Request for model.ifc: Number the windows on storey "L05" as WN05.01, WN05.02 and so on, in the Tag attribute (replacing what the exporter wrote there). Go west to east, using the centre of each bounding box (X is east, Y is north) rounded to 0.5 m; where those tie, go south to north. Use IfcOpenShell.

First a look at what the model holds.

```python
import ifcopenshell
import ifcopenshell.util.element
import ifcopenshell.util.placement

model = ifcopenshell.open("model.ifc")
print(model.schema)
storey = next(s for s in model.by_type("IfcBuildingStorey") if s.Name == "L05")
windows = [e for e in ifcopenshell.util.element.get_decomposition(storey) if e.is_a("IfcWindow")]
for e in sorted(windows, key=lambda e: e.id()):
    origin = ifcopenshell.util.placement.get_local_placement(e.ObjectPlacement)[:3, 3]
    print(e.id(), e.Tag, e.Name, origin.round(2) + 0.0, sep=" | ")
```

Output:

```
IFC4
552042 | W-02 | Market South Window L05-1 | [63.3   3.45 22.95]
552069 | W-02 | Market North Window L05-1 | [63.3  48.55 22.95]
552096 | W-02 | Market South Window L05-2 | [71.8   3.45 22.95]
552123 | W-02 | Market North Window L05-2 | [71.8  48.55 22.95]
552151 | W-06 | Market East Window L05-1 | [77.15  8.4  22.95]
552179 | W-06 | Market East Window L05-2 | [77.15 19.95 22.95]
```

```python
import ifcopenshell
import ifcopenshell.geom
import ifcopenshell.util.element
import ifcopenshell.util.shape

model = ifcopenshell.open("model.ifc")
settings = ifcopenshell.geom.settings()
settings.set("use-world-coords", True)


def centre(element):
    shape = ifcopenshell.geom.create_shape(settings, element)
    return ifcopenshell.util.shape.get_bbox_centroid(shape.geometry)


storey = next(s for s in model.by_type("IfcBuildingStorey") if s.Name == "L05")
windows = [e for e in ifcopenshell.util.element.get_decomposition(storey) if e.is_a("IfcWindow")]

# Insertion points can sit at a corner or the storey origin, so sort by the geometry (in metres).
centres = {e: centre(e) for e in windows}
windows.sort(key=lambda e: (round(centres[e][0] / 0.5), centres[e][1]))

for i, e in enumerate(windows, start=1):
    number = f"WN05.{i:02d}"
    e.Tag = number
    print(e.id(), number)

model.write("model_v2.ifc")
```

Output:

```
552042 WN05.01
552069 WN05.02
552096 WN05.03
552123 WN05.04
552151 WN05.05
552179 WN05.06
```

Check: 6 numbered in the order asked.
